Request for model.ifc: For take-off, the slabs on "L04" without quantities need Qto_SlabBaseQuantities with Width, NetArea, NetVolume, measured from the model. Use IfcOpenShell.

First a look at what the model holds.

```python
import ifcopenshell
import ifcopenshell.util.element
import ifcopenshell.util.unit

model = ifcopenshell.open("model.ifc")
print(model.schema)
for unit_type in ("LENGTHUNIT", "AREAUNIT", "VOLUMEUNIT"):
    print(unit_type, ifcopenshell.util.unit.calculate_unit_scale(model, unit_type))
storey = next(s for s in model.by_type("IfcBuildingStorey") if s.Name == "L04")
slabs = [e for e in ifcopenshell.util.element.get_decomposition(storey) if e.is_a("IfcSlab")]
for e in sorted(slabs, key=lambda e: e.id()):
    print(e.id(), e.is_a(), e.Name, list(ifcopenshell.util.element.get_psets(e, qtos_only=True)), sep=" | ")
```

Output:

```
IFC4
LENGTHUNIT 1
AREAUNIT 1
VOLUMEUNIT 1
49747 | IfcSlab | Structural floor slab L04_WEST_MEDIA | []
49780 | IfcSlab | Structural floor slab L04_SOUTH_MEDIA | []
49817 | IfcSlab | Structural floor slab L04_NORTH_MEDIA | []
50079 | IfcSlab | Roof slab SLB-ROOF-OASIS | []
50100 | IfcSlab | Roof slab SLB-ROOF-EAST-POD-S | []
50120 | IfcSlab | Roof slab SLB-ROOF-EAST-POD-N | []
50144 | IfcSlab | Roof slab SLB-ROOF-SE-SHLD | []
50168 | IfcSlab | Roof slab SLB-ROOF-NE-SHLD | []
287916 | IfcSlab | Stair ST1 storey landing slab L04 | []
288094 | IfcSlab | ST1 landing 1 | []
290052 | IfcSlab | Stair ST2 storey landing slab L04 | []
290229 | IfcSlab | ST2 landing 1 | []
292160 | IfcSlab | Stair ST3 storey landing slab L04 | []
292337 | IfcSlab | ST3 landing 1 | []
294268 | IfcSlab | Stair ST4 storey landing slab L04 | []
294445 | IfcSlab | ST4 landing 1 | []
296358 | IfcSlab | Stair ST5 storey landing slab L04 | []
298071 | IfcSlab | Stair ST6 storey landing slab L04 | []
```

```python
import ifcopenshell
import ifcopenshell.api.pset
import ifcopenshell.geom
import ifcopenshell.util.element
import ifcopenshell.util.shape
import ifcopenshell.util.unit

model = ifcopenshell.open("model.ifc")
unit_scale = ifcopenshell.util.unit.calculate_unit_scale(model)
area_scale = ifcopenshell.util.unit.calculate_unit_scale(model, "AREAUNIT")
volume_scale = ifcopenshell.util.unit.calculate_unit_scale(model, "VOLUMEUNIT")
settings = ifcopenshell.geom.settings()

storey = next(s for s in model.by_type("IfcBuildingStorey") if s.Name == "L04")
slabs = [e for e in ifcopenshell.util.element.get_decomposition(storey) if e.is_a("IfcSlab")]

for e in sorted(slabs, key=lambda e: e.id()):
    if ifcopenshell.util.element.get_psets(e, qtos_only=True, should_inherit=False):
        continue
    # Geometry comes back in metres, in the element's own axes.
    shape = ifcopenshell.geom.create_shape(settings, e)
    values = {
        "Width": ifcopenshell.util.shape.get_z(shape.geometry) / unit_scale,
        "NetArea": ifcopenshell.util.shape.get_footprint_area(shape.geometry) / area_scale,
        "NetVolume": ifcopenshell.util.shape.get_volume(shape.geometry) / volume_scale,
    }
    qto = ifcopenshell.api.pset.add_qto(model, product=e, name="Qto_SlabBaseQuantities")
    ifcopenshell.api.pset.edit_qto(model, qto=qto, properties=values)
    print(e.id(), {k: round(v, 3) for k, v in values.items()})

model.write("model_edited.ifc")
```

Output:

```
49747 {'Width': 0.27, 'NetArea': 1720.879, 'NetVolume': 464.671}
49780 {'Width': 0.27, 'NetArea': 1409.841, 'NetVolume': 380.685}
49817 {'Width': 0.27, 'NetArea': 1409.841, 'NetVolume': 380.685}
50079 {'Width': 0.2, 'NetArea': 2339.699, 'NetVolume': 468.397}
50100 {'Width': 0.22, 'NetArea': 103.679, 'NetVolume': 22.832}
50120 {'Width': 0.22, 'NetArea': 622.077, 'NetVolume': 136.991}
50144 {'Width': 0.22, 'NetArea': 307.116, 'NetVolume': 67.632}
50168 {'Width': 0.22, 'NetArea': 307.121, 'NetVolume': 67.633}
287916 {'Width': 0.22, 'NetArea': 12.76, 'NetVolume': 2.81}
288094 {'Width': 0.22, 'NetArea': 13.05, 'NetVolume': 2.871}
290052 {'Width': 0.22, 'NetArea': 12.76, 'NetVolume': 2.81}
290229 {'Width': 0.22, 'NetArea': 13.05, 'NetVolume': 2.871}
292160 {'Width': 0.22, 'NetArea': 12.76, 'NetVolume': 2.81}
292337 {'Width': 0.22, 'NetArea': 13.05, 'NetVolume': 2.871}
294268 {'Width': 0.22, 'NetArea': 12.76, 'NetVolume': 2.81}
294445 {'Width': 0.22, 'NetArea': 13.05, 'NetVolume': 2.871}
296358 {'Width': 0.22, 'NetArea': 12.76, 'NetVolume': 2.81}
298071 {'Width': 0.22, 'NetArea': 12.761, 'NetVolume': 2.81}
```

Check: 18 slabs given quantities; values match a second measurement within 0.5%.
